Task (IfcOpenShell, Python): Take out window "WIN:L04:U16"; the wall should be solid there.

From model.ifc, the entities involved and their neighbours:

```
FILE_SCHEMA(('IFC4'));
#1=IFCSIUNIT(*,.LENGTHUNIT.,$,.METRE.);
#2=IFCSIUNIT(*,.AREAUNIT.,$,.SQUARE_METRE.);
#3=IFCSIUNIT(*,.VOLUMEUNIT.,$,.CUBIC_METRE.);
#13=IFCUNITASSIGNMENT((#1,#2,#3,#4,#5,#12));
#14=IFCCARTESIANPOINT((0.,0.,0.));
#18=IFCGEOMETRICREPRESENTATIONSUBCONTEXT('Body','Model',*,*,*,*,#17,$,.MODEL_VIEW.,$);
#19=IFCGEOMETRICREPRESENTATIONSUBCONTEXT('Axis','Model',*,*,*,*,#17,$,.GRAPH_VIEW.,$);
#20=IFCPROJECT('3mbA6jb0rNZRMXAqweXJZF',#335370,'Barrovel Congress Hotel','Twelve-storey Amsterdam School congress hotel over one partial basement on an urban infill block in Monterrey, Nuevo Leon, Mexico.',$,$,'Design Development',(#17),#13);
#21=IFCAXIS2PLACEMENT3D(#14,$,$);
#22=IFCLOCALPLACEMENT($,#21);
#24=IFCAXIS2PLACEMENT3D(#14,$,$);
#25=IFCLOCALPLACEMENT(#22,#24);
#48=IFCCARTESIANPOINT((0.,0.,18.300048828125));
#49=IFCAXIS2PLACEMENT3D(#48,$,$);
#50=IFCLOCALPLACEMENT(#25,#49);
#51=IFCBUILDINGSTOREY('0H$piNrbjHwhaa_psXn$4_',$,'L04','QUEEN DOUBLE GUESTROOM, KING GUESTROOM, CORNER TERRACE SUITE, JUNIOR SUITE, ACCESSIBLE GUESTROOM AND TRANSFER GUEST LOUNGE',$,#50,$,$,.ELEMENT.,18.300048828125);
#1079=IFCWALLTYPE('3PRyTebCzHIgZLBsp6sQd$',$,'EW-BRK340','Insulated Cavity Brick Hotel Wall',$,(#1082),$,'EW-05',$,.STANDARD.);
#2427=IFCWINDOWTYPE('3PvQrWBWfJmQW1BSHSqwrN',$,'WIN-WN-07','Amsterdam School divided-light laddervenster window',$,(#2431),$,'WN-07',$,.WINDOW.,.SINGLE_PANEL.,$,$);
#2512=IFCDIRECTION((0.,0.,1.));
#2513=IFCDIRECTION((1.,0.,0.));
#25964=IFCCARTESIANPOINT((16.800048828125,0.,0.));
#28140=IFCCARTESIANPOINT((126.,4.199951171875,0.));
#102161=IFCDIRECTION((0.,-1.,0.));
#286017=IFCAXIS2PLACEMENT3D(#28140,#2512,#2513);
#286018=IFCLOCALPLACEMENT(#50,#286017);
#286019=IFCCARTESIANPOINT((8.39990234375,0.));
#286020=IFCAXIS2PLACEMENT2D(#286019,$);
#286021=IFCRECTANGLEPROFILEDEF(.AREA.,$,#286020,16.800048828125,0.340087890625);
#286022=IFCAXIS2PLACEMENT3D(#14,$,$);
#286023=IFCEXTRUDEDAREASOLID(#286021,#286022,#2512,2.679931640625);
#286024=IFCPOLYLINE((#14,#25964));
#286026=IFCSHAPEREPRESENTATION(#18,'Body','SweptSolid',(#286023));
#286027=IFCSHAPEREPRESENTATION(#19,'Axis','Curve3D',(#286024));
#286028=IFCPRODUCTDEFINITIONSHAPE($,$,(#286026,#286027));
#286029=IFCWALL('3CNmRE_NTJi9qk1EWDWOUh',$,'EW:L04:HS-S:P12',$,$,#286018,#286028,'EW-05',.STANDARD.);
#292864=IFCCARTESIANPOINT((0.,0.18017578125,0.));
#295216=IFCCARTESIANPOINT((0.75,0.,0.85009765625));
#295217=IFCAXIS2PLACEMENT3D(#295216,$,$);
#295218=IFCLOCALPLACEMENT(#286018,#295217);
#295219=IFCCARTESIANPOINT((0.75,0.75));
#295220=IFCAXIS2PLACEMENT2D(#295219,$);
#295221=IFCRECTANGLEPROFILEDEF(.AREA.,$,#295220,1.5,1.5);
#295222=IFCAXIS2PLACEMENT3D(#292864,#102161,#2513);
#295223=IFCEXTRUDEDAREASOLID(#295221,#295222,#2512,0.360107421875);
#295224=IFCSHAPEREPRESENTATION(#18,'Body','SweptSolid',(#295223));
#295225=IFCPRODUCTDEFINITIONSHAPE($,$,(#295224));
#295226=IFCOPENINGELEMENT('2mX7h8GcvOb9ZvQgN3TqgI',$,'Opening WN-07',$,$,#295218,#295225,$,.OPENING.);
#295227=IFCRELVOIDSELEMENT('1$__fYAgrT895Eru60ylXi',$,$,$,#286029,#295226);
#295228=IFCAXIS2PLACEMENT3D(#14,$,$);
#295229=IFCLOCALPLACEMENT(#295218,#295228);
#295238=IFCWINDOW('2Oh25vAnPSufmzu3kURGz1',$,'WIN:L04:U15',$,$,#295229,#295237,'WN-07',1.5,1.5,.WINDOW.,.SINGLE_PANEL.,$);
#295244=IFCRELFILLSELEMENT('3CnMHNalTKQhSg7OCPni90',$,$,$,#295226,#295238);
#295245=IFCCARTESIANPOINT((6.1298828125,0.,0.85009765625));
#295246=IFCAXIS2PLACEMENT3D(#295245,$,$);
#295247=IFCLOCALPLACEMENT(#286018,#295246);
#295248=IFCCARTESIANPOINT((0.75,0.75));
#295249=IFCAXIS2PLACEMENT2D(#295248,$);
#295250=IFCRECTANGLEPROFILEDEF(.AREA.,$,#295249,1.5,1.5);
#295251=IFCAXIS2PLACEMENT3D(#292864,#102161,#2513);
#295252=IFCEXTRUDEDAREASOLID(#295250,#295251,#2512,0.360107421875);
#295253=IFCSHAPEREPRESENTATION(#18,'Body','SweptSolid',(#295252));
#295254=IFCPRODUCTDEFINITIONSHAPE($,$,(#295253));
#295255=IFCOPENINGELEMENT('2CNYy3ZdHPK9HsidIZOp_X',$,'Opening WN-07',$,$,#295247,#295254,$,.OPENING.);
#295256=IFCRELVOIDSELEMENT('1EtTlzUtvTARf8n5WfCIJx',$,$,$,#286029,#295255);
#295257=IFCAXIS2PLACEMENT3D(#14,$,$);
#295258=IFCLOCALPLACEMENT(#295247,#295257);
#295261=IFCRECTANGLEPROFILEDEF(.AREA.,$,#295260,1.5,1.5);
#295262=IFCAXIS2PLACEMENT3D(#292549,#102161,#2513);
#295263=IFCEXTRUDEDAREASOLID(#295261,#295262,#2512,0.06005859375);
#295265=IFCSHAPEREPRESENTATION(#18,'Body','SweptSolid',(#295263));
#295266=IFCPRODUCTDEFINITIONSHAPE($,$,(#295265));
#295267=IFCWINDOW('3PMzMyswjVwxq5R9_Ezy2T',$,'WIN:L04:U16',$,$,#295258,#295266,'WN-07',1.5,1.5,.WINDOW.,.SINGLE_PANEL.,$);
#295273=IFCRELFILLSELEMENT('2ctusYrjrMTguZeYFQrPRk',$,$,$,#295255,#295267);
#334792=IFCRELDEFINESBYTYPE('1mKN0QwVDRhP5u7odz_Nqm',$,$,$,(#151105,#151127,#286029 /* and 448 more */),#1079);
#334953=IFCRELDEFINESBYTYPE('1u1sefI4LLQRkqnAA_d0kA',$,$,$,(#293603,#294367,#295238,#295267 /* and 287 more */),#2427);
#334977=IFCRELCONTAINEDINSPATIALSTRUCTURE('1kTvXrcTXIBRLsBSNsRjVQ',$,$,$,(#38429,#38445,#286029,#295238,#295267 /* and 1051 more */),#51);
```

```python
import ifcopenshell
import ifcopenshell.api.feature
import ifcopenshell.api.root
import ifcopenshell.geom
import ifcopenshell.util.shape

model = ifcopenshell.open("model.ifc")
settings = ifcopenshell.geom.settings()


def volume(element):
    """Net volume in cubic metres, openings subtracted."""
    shape = ifcopenshell.geom.create_shape(settings, element)
    return ifcopenshell.util.shape.get_volume(shape.geometry)


window = model.by_id(295267)
opening = window.FillsVoids[0].RelatingOpeningElement
wall = opening.VoidsElements[0].RelatingBuildingElement
before = volume(wall)

ifcopenshell.api.root.remove_product(model, product=window)
ifcopenshell.api.feature.remove_feature(model, feature=opening)

after = volume(wall)

print(f"wall volume {before:.3f} -> {after:.3f} m3")

model.write("model_v2.ifc")
```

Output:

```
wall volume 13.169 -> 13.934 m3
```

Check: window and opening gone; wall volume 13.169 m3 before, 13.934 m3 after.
